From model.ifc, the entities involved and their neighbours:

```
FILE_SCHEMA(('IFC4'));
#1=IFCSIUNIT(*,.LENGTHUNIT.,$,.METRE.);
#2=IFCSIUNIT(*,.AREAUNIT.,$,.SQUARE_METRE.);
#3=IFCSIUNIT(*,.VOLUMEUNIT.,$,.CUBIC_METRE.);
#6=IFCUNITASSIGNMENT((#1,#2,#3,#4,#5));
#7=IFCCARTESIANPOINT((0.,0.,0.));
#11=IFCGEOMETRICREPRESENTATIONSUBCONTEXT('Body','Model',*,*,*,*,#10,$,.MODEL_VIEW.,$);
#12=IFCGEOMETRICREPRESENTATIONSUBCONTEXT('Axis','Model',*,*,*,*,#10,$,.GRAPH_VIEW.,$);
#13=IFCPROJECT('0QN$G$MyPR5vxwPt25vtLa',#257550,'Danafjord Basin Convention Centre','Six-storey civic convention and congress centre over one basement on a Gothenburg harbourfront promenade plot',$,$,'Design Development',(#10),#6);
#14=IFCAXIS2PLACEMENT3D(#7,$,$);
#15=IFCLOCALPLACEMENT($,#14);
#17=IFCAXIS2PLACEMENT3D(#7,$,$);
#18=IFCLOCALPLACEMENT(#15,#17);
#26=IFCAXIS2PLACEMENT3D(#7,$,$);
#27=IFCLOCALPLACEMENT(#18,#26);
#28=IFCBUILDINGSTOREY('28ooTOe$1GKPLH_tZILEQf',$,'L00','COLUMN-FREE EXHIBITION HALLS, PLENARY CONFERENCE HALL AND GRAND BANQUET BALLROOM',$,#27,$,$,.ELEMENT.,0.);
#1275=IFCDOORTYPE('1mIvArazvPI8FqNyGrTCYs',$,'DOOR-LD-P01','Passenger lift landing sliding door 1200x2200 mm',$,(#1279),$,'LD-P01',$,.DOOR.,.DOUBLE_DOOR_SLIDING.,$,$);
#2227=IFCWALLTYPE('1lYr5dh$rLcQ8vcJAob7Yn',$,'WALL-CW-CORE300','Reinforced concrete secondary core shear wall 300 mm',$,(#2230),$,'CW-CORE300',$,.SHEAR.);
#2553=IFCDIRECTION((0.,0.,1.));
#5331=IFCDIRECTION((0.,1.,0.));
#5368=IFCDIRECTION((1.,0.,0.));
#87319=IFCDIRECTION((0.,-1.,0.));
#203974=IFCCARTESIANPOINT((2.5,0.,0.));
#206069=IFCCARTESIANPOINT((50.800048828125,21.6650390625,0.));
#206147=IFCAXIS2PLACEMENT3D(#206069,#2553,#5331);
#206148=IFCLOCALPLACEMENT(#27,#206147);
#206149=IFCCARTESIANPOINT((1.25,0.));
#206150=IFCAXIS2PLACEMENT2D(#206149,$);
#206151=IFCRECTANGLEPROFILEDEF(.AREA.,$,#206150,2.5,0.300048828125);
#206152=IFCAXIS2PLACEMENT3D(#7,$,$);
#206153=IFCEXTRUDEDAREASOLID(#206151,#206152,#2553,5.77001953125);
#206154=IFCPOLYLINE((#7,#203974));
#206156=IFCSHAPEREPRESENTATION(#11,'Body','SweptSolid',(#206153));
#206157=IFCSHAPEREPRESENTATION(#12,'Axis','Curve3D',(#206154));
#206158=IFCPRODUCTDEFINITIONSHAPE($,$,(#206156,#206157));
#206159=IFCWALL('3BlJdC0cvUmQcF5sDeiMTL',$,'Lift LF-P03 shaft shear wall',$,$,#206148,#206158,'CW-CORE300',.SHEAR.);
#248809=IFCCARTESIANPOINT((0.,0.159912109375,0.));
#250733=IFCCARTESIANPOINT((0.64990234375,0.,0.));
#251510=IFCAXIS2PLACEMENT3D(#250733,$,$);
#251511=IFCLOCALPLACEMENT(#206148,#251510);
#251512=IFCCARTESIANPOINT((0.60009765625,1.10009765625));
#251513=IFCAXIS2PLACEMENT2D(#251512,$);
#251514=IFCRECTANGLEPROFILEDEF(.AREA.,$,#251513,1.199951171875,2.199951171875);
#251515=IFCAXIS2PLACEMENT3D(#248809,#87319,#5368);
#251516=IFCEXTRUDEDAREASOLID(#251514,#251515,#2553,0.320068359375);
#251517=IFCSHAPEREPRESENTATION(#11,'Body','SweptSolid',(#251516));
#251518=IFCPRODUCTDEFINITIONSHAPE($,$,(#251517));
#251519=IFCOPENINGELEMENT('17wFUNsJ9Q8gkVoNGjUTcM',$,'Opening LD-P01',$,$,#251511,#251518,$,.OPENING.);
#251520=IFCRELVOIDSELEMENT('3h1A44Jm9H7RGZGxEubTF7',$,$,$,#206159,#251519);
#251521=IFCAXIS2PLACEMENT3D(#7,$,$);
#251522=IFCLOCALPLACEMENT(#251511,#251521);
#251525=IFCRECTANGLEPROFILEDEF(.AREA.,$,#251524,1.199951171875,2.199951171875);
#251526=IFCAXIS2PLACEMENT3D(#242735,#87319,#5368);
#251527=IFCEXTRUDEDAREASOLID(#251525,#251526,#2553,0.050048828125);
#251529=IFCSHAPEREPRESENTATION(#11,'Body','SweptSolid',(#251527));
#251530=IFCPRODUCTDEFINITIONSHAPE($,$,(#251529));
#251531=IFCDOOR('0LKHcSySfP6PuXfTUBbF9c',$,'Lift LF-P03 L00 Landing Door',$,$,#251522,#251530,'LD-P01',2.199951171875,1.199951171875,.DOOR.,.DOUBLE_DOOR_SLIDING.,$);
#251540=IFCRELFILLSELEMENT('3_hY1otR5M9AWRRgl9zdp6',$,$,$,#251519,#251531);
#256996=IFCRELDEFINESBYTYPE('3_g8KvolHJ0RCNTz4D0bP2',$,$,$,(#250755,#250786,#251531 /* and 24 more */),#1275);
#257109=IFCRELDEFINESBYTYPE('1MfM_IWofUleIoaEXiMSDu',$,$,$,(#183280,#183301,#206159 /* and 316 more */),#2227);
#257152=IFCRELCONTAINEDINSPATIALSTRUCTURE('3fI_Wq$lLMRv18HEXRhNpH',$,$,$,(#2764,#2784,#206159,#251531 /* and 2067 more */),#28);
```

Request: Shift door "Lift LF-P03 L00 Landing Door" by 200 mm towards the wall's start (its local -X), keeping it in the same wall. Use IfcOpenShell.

```python
import ifcopenshell
import ifcopenshell.api.geometry
import ifcopenshell.util.placement

model = ifcopenshell.open("model.ifc")

door = model.by_id(251531)
opening = door.FillsVoids[0].RelatingOpeningElement
wall = opening.VoidsElements[0].RelatingBuildingElement

wall_matrix = ifcopenshell.util.placement.get_local_placement(wall.ObjectPlacement)
shift = wall_matrix[:3, 0] * -0.2
before = ifcopenshell.util.placement.get_local_placement(door.ObjectPlacement)[:3, 3].copy()

# The door is placed relative to its opening, so it follows when the opening moves.
matrix = ifcopenshell.util.placement.get_local_placement(opening.ObjectPlacement)
matrix[:3, 3] += shift
ifcopenshell.api.geometry.edit_object_placement(
    model, product=opening, matrix=matrix, is_si=False, should_transform_children=True
)

after = ifcopenshell.util.placement.get_local_placement(door.ObjectPlacement)[:3, 3]
print("door moved by", (after - before).round(3) + 0.0)

model.write("model_v2.ifc")
```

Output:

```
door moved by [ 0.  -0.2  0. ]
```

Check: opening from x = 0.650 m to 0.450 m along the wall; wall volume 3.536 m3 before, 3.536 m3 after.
